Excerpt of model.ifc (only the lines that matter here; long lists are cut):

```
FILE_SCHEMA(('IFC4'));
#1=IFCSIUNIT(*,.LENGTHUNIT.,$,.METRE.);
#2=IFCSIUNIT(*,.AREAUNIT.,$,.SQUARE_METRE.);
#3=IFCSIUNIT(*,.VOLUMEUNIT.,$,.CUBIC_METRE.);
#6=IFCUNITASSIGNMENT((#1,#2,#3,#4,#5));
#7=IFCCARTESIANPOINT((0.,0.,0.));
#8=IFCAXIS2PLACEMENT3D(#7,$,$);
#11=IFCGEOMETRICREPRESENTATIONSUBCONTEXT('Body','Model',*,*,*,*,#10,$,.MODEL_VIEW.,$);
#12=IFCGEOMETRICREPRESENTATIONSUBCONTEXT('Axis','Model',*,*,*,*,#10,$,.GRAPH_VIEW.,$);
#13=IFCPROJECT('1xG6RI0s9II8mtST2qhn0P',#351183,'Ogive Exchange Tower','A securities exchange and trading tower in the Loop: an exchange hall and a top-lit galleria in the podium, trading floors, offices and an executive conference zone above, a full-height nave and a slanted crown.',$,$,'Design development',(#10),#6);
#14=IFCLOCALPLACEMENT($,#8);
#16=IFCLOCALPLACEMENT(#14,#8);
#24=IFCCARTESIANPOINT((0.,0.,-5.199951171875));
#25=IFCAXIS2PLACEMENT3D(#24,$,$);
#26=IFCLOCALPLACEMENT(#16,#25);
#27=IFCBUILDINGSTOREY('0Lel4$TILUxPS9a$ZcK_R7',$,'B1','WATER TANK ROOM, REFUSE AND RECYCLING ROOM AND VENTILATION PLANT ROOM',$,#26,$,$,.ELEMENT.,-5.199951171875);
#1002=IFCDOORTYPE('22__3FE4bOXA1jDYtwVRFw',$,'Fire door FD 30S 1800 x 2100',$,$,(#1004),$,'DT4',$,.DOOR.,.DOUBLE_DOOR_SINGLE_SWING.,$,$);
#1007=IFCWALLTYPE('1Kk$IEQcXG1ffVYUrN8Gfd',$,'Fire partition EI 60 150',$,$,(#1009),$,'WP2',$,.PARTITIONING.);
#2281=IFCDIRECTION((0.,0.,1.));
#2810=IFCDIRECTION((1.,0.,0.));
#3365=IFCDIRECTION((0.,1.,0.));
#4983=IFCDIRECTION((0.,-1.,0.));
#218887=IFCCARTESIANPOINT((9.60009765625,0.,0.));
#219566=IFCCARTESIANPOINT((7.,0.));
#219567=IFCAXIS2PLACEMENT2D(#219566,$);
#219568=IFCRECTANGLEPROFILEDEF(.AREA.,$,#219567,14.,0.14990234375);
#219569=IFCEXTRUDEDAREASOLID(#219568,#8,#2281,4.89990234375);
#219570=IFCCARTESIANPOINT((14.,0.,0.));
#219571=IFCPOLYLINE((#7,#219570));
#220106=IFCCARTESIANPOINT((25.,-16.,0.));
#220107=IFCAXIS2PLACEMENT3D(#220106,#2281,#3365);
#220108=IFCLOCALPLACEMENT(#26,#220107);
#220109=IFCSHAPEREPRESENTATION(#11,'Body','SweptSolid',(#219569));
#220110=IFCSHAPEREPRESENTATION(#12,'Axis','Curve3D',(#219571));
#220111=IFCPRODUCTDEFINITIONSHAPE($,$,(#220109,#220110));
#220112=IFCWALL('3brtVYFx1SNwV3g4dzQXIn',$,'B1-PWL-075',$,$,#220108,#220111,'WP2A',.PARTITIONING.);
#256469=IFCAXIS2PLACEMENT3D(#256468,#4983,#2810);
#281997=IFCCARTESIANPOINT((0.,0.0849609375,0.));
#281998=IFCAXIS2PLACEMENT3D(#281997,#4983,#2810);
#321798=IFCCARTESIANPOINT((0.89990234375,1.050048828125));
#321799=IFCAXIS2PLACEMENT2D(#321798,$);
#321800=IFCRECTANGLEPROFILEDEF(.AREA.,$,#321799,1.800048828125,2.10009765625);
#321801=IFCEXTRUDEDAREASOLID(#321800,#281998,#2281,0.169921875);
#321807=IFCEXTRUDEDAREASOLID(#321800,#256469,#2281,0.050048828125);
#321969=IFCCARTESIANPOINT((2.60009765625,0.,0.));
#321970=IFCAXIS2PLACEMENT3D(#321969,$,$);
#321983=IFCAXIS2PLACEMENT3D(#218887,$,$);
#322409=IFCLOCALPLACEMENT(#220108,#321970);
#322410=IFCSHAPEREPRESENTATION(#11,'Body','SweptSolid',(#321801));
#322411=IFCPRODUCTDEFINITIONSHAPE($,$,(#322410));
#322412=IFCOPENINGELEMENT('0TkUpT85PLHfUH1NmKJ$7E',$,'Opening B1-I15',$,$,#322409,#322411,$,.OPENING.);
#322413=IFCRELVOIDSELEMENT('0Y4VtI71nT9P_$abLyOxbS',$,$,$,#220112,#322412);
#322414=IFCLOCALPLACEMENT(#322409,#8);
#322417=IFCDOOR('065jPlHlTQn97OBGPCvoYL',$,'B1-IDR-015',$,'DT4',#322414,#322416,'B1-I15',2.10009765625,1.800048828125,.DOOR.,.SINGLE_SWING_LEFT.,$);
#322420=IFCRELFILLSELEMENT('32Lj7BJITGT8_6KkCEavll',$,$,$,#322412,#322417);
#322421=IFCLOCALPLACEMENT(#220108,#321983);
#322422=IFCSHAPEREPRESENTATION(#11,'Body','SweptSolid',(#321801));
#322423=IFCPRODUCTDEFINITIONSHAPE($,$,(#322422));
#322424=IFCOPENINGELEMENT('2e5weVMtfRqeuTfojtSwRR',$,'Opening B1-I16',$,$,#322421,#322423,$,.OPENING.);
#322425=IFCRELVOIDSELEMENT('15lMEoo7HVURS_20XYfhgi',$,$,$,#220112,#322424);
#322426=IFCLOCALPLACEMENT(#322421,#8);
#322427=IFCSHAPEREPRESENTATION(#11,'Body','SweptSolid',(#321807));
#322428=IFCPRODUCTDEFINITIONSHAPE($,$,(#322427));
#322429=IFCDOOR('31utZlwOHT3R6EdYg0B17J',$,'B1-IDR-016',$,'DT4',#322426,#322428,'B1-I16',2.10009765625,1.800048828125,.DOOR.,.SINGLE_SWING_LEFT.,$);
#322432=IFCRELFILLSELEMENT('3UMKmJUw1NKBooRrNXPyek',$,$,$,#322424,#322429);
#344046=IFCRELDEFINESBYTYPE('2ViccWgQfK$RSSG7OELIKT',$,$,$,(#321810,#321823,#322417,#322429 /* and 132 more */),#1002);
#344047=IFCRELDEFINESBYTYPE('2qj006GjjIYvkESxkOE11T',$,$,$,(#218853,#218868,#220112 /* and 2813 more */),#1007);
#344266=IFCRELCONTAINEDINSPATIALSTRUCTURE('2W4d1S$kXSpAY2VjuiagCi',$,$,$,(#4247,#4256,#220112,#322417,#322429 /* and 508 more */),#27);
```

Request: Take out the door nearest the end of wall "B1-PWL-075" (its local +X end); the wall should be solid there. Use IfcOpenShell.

```python
import ifcopenshell
import ifcopenshell.api.feature
import ifcopenshell.api.root
import ifcopenshell.geom
import ifcopenshell.util.shape

model = ifcopenshell.open("model.ifc")
settings = ifcopenshell.geom.settings()


def volume(element):
    """Net volume in cubic metres, openings subtracted."""
    shape = ifcopenshell.geom.create_shape(settings, element)
    return ifcopenshell.util.shape.get_volume(shape.geometry)


door = model.by_guid("31utZlwOHT3R6EdYg0B17J")
opening = door.FillsVoids[0].RelatingOpeningElement
wall = opening.VoidsElements[0].RelatingBuildingElement
before = volume(wall)

ifcopenshell.api.root.remove_product(model, product=door)
ifcopenshell.api.feature.remove_feature(model, feature=opening)

after = volume(wall)

print(f"wall volume {before:.3f} -> {after:.3f} m3")

model.write("model_rev.ifc")
```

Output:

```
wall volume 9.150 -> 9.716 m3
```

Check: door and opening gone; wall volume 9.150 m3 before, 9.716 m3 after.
